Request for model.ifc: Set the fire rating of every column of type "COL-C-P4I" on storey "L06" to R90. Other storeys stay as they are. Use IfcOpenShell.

First a look at what the model holds.

```python
import ifcopenshell
import ifcopenshell.util.element

model = ifcopenshell.open("model.ifc")
print(model.schema)
storey = next(s for s in model.by_type("IfcBuildingStorey") if s.Name == "L06")
columns = [e for e in ifcopenshell.util.element.get_decomposition(storey) if e.is_a("IfcColumn")]
seen = {}
for e in columns:
    element_type = ifcopenshell.util.element.get_type(e)
    key = (element_type.Name if element_type != e and element_type else None, ifcopenshell.util.element.get_pset(e, "Pset_ColumnCommon", "FireRating"))
    seen[key] = seen.get(key, 0) + 1
for (name, value), count in sorted(seen.items(), key=str):
    print(count, "x", name, "|", value)
```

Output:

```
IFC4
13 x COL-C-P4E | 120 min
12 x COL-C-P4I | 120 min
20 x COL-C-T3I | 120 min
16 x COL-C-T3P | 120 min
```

```python
import ifcopenshell
import ifcopenshell.api.pset
import ifcopenshell.util.element

model = ifcopenshell.open("model.ifc")

storey = next(s for s in model.by_type("IfcBuildingStorey") if s.Name == "L06")
columns = [e for e in ifcopenshell.util.element.get_decomposition(storey) if e.is_a("IfcColumn")]

count = 0
for e in columns:
    element_type = ifcopenshell.util.element.get_type(e)
    if element_type in (None, e) or element_type.Name != "COL-C-P4I":
        continue
    # add_pset returns the element's existing set when there is one.
    pset = ifcopenshell.api.pset.add_pset(model, product=e, name="Pset_ColumnCommon")
    ifcopenshell.api.pset.edit_pset(model, pset=pset, properties={"FireRating": "R90"})
    count += 1

print(count, "columns updated")

model.write("model-out.ifc")
```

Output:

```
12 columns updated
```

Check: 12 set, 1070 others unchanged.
